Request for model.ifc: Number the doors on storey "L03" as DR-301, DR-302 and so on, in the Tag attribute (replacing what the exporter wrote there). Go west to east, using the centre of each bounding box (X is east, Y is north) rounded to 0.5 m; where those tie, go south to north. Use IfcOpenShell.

First a look at what the model holds.

```python
import ifcopenshell
import ifcopenshell.util.element
import ifcopenshell.util.placement

model = ifcopenshell.open("model.ifc")
print(model.schema)
storey = next(s for s in model.by_type("IfcBuildingStorey") if s.Name == "L03")
doors = [e for e in ifcopenshell.util.element.get_decomposition(storey) if e.is_a("IfcDoor")]
for e in sorted(doors, key=lambda e: e.id()):
    origin = ifcopenshell.util.placement.get_local_placement(e.ObjectPlacement)[:3, 3]
    print(e.id(), e.Tag, e.Name, origin.round(2) + 0.0, sep=" | ")
```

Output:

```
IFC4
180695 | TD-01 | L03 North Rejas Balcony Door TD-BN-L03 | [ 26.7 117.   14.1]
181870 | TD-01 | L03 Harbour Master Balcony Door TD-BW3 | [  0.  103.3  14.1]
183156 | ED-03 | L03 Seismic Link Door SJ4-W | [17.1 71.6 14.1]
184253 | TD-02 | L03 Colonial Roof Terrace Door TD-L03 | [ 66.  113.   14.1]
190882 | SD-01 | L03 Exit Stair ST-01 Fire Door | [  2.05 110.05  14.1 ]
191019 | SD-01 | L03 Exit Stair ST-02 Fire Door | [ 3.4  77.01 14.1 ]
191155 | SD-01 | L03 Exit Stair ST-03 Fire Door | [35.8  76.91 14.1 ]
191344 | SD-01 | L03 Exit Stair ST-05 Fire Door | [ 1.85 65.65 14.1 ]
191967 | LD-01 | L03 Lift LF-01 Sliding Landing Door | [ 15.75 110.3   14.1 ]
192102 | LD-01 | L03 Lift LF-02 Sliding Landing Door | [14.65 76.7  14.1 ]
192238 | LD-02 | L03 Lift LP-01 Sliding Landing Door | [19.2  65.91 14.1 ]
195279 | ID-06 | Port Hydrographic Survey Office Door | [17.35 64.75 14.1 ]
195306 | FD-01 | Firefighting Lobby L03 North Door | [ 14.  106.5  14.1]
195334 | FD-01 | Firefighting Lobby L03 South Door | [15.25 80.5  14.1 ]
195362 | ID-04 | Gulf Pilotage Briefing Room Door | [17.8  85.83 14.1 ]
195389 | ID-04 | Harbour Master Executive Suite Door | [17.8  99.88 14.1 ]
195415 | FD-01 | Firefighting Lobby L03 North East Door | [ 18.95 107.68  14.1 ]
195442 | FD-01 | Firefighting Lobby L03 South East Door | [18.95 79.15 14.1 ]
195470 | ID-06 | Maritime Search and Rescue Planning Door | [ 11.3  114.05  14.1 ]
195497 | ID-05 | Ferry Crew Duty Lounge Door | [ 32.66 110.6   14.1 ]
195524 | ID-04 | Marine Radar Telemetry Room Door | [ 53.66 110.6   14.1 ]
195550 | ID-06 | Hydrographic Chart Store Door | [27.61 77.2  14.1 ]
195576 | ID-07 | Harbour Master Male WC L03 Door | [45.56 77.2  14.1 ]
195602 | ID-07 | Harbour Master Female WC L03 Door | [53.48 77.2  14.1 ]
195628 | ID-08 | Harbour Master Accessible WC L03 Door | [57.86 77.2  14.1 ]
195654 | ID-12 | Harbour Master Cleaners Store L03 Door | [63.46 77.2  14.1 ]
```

```python
import ifcopenshell
import ifcopenshell.geom
import ifcopenshell.util.element
import ifcopenshell.util.shape

model = ifcopenshell.open("model.ifc")
settings = ifcopenshell.geom.settings()
settings.set("use-world-coords", True)


def centre(element):
    shape = ifcopenshell.geom.create_shape(settings, element)
    return ifcopenshell.util.shape.get_bbox_centroid(shape.geometry)


storey = next(s for s in model.by_type("IfcBuildingStorey") if s.Name == "L03")
doors = [e for e in ifcopenshell.util.element.get_decomposition(storey) if e.is_a("IfcDoor")]

# Insertion points can sit at a corner or the storey origin, so sort by the geometry (in metres).
centres = {e: centre(e) for e in doors}
doors.sort(key=lambda e: (round(centres[e][0] / 0.5), centres[e][1]))

for i, e in enumerate(doors, start=1):
    number = f"DR-3{i:02d}"
    e.Tag = number
    print(e.id(), number)

model.write("model_updated.ifc")
```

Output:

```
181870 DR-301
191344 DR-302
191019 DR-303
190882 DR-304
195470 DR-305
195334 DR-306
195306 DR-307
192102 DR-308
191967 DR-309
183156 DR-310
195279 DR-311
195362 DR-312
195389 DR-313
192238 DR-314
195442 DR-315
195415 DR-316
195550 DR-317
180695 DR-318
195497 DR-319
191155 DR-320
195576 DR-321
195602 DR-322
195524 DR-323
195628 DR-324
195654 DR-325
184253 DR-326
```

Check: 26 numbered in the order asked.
